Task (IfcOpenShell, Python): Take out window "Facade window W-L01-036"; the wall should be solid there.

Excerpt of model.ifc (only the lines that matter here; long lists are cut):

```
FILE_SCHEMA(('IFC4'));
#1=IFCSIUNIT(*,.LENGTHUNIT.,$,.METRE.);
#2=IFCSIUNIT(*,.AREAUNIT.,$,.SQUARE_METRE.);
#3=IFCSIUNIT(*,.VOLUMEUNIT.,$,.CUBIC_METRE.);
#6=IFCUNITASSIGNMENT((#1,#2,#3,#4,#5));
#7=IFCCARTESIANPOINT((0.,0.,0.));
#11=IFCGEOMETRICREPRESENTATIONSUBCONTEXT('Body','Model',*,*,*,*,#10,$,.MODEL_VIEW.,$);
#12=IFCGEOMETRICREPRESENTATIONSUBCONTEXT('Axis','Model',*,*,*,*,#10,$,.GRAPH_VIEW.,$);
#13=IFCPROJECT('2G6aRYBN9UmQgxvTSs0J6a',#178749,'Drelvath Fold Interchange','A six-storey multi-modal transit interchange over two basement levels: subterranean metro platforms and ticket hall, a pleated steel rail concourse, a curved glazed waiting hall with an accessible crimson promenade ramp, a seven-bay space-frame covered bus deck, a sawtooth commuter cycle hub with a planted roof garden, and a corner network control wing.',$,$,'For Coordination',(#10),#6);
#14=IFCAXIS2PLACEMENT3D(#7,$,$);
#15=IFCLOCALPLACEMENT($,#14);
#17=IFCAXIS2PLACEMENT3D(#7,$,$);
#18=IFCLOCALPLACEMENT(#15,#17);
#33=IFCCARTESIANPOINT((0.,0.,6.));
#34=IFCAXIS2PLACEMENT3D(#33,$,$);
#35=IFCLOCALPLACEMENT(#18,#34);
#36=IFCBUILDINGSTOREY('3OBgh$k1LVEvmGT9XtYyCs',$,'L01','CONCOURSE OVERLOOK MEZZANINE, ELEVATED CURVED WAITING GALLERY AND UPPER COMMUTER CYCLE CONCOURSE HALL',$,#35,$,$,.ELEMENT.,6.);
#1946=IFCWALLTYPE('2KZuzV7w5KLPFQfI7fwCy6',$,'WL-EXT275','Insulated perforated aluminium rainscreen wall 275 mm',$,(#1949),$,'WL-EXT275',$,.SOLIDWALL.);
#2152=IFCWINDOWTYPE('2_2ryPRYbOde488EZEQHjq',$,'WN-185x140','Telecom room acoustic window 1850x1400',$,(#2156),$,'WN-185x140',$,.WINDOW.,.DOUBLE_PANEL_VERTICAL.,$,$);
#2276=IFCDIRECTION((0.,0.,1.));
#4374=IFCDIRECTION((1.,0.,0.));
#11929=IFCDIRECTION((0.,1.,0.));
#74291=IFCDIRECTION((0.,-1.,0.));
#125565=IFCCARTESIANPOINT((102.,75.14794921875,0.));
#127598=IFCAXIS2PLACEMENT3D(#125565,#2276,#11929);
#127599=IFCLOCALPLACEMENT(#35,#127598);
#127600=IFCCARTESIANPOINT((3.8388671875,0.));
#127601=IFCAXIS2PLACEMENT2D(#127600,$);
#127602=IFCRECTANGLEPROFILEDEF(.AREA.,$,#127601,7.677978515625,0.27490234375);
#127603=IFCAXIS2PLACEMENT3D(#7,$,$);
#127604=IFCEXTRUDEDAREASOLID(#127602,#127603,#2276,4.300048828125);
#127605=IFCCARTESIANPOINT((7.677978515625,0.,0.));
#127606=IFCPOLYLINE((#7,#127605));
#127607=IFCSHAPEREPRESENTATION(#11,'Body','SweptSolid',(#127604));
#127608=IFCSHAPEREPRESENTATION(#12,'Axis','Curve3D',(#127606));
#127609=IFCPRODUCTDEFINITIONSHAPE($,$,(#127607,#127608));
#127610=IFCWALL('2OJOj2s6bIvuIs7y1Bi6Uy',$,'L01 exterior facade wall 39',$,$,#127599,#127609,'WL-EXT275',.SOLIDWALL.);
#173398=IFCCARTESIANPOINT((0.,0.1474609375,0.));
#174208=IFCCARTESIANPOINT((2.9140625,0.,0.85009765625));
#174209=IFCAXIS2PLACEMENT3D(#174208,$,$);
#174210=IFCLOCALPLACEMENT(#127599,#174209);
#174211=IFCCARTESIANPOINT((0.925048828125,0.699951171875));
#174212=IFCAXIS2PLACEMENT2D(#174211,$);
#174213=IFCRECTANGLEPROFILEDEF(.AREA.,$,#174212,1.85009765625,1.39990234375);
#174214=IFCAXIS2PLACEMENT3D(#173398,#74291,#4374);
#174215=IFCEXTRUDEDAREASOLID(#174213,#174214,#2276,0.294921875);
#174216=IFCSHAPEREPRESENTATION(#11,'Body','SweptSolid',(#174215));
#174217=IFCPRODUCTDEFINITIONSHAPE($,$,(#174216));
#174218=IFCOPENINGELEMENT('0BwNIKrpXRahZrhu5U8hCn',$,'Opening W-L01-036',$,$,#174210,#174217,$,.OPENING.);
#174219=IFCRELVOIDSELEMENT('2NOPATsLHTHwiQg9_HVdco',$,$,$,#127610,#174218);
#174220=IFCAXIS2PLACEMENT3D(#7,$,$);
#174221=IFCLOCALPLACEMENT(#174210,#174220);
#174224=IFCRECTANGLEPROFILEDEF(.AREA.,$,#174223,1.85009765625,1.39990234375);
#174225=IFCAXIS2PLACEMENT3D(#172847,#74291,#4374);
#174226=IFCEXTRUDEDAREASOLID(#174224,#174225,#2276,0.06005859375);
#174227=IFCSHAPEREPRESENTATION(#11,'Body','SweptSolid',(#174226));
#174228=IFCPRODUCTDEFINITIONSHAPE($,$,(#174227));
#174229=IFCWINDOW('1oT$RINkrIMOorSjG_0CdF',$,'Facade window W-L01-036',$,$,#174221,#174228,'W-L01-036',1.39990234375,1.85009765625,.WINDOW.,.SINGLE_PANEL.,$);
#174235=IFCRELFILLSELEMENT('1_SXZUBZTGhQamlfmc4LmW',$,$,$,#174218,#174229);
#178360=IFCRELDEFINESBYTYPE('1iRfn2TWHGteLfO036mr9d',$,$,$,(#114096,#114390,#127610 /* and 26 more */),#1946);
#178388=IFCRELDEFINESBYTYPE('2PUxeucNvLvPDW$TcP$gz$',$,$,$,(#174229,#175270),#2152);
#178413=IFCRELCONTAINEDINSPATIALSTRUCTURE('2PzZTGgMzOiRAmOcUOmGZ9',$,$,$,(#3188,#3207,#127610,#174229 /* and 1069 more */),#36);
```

```python
import ifcopenshell
import ifcopenshell.api.feature
import ifcopenshell.api.root
import ifcopenshell.geom
import ifcopenshell.util.shape

model = ifcopenshell.open("model.ifc")
settings = ifcopenshell.geom.settings()


def volume(element):
    """Net volume in cubic metres, openings subtracted."""
    shape = ifcopenshell.geom.create_shape(settings, element)
    return ifcopenshell.util.shape.get_volume(shape.geometry)


window = model.by_id(174229)
opening = window.FillsVoids[0].RelatingOpeningElement
wall = opening.VoidsElements[0].RelatingBuildingElement
before = volume(wall)

ifcopenshell.api.root.remove_product(model, product=window)
ifcopenshell.api.feature.remove_feature(model, feature=opening)

after = volume(wall)

print(f"wall volume {before:.3f} -> {after:.3f} m3")

model.write("model_edited.ifc")
```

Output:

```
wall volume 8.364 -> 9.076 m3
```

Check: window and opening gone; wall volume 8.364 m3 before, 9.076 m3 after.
